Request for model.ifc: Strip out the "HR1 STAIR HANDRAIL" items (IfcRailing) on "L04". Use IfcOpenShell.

First a look at what the model holds.

```python
import ifcopenshell
import ifcopenshell.util.element

model = ifcopenshell.open("model.ifc")
print(model.schema)
storey = next(s for s in model.by_type("IfcBuildingStorey") if s.Name == "L04")
railings = [e for e in ifcopenshell.util.element.get_decomposition(storey) if e.is_a("IfcRailing")]
seen = {}
for e in railings:
    element_type = ifcopenshell.util.element.get_type(e)
    name = element_type.Name if element_type not in (None, e) else None
    seen[name] = seen.get(name, 0) + 1
for name, count in sorted(seen.items(), key=str):
    print(count, "x", name)
```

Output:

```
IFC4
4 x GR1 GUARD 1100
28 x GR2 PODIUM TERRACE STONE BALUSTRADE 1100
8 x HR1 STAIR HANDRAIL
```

```python
import ifcopenshell
import ifcopenshell.api.root
import ifcopenshell.util.element

model = ifcopenshell.open("model.ifc")

storey = next(s for s in model.by_type("IfcBuildingStorey") if s.Name == "L04")
railings = [e for e in ifcopenshell.util.element.get_decomposition(storey) if e.is_a("IfcRailing")]
targets = [e for e in railings if (t := ifcopenshell.util.element.get_type(e)) not in (None, e) and t.Name == "HR1 STAIR HANDRAIL"]

for e in targets:
    ifcopenshell.api.root.remove_product(model, product=e)
print(len(targets), "removed")

model.write("model_rev.ifc")
```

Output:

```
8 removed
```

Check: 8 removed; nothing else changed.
